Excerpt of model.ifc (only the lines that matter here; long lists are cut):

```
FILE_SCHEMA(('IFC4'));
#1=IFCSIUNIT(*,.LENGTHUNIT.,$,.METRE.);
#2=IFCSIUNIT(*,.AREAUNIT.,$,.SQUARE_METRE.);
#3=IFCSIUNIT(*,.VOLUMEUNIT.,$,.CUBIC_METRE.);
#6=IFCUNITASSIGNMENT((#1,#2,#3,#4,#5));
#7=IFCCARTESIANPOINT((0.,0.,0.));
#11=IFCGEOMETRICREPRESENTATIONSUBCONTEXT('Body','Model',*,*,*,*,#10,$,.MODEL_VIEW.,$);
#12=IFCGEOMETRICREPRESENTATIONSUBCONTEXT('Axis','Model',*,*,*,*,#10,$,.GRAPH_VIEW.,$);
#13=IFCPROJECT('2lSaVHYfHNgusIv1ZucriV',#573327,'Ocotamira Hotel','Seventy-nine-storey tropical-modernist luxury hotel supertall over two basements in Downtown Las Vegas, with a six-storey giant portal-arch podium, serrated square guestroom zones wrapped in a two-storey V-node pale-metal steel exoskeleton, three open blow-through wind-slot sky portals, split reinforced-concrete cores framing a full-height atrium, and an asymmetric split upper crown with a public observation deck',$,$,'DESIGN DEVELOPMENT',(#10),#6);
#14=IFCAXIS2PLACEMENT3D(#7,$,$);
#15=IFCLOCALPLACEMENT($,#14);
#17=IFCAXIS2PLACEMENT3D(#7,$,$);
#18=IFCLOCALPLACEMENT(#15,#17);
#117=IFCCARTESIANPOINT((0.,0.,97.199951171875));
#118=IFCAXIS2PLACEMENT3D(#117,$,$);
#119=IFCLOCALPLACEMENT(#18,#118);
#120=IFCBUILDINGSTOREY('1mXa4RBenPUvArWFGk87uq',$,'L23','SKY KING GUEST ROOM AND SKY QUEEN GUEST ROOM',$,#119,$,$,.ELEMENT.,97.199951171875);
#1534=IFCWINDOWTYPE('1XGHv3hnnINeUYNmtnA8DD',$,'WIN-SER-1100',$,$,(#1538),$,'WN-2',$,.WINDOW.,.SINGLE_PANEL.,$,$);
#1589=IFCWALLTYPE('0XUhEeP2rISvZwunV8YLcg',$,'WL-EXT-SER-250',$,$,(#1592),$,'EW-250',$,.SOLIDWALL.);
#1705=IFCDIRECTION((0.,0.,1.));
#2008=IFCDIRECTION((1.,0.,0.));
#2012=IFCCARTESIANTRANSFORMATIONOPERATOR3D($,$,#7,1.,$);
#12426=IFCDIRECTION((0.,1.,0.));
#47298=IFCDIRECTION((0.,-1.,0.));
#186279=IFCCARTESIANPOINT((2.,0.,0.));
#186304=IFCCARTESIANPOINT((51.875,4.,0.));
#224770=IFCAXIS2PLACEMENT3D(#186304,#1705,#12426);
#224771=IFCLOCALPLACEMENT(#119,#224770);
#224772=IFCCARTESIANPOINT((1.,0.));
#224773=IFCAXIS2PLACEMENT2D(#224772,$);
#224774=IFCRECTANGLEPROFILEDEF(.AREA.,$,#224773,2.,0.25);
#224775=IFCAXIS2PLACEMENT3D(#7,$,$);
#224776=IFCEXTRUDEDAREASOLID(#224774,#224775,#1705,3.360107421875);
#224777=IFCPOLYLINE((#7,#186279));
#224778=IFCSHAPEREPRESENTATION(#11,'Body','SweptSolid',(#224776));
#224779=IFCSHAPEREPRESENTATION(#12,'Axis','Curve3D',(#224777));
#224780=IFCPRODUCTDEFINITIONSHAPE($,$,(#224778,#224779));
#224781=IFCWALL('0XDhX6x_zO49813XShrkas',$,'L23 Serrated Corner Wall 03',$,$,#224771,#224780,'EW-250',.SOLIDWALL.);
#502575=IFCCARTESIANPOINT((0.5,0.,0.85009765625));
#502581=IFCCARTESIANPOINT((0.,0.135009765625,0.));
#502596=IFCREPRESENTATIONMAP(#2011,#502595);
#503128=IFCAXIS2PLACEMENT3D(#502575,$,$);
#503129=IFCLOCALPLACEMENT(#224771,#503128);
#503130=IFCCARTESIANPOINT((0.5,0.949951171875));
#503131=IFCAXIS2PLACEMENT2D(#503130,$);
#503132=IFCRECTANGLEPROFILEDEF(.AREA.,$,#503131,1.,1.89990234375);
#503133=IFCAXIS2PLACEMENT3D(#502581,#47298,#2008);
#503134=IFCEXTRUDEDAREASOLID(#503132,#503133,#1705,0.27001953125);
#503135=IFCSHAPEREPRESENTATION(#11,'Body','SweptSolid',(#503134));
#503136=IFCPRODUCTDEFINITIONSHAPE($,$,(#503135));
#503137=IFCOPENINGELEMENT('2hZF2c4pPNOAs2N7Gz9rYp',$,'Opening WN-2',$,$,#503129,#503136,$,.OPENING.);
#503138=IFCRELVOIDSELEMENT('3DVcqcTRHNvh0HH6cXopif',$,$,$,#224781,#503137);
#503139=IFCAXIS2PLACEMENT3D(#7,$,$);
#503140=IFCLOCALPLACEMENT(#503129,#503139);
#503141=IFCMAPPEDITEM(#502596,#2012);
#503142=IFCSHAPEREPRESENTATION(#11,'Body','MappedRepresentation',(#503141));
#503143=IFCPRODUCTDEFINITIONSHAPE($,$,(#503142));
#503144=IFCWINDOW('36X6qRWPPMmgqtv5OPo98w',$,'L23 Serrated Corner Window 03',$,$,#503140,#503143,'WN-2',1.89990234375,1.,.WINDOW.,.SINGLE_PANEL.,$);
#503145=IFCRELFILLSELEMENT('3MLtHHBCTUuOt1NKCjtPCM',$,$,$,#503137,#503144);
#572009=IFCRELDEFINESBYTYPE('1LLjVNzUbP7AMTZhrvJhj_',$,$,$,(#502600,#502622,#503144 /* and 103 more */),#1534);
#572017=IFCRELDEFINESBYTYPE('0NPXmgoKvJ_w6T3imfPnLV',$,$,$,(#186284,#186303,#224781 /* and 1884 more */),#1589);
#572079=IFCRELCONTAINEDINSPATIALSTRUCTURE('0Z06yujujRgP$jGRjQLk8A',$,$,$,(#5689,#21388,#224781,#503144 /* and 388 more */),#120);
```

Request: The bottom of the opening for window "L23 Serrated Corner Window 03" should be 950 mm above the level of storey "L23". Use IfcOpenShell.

```python
import numpy as np
import ifcopenshell
import ifcopenshell.api.geometry
import ifcopenshell.geom
import ifcopenshell.util.element
import ifcopenshell.util.placement
import ifcopenshell.util.shape
import ifcopenshell.util.unit

model = ifcopenshell.open("model.ifc")
unit_scale = ifcopenshell.util.unit.calculate_unit_scale(model)

window = model.by_guid("36X6qRWPPMmgqtv5OPo98w")
opening = window.FillsVoids[0].RelatingOpeningElement
storey = ifcopenshell.util.element.get_container(window, ifc_class="IfcBuildingStorey")
level = ifcopenshell.util.placement.get_local_placement(storey.ObjectPlacement)[2, 3]

# The opening's origin need not be at the sill, so measure its lowest point.
shape = ifcopenshell.geom.create_shape(ifcopenshell.geom.settings(), opening)
bottom = ifcopenshell.util.shape.get_shape_bottom_elevation(shape, shape.geometry) / unit_scale
dz = level + 0.95 / unit_scale - bottom

shift = np.array([0.0, 0.0, dz])
# The window is placed relative to its opening, so it follows when the opening moves.
matrix = ifcopenshell.util.placement.get_local_placement(opening.ObjectPlacement)
matrix[:3, 3] += shift
ifcopenshell.api.geometry.edit_object_placement(
    model, product=opening, matrix=matrix, is_si=False, should_transform_children=True
)

print(f"moved by {dz * unit_scale:+.3f} m")

model.write("model_rev.ifc")
```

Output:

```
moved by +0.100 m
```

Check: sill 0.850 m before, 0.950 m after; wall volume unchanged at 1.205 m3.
